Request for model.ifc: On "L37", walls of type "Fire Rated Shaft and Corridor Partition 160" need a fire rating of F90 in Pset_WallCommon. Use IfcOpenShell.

First a look at what the model holds.

```python
import ifcopenshell
import ifcopenshell.util.element

model = ifcopenshell.open("model.ifc")
print(model.schema)
storey = next(s for s in model.by_type("IfcBuildingStorey") if s.Name == "L37")
walls = [e for e in ifcopenshell.util.element.get_decomposition(storey) if e.is_a("IfcWall")]
seen = {}
for e in walls:
    element_type = ifcopenshell.util.element.get_type(e)
    key = (element_type.Name if element_type != e and element_type else None, ifcopenshell.util.element.get_pset(e, "Pset_WallCommon", "FireRating"))
    seen[key] = seen.get(key, 0) + 1
for (name, value), count in sorted(seen.items(), key=str):
    print(count, "x", name, "|", value)
```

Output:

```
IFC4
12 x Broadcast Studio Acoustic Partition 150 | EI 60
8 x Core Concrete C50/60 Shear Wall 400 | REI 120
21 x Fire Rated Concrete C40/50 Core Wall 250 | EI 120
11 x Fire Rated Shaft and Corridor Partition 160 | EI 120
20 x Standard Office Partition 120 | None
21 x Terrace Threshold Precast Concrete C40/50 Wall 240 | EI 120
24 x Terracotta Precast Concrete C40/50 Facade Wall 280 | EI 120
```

```python
import ifcopenshell
import ifcopenshell.api.pset
import ifcopenshell.util.element

model = ifcopenshell.open("model.ifc")

storey = next(s for s in model.by_type("IfcBuildingStorey") if s.Name == "L37")
walls = [e for e in ifcopenshell.util.element.get_decomposition(storey) if e.is_a("IfcWall")]

count = 0
for e in walls:
    element_type = ifcopenshell.util.element.get_type(e)
    if element_type in (None, e) or element_type.Name != "Fire Rated Shaft and Corridor Partition 160":
        continue
    found = ifcopenshell.util.element.get_pset(e, "Pset_WallCommon", should_inherit=False)
    if found:
        pset = model.by_id(found["id"])
        if len(ifcopenshell.util.element.get_elements_by_pset(pset)) > 1:
            pset = ifcopenshell.api.pset.unshare_pset(model, products=[e], pset=pset)[0]
    else:
        pset = ifcopenshell.api.pset.add_pset(model, product=e, name="Pset_WallCommon")
    ifcopenshell.api.pset.edit_pset(model, pset=pset, properties={"FireRating": "F90"})
    count += 1

print(count, "walls updated")

model.write("model_v2.ifc")
```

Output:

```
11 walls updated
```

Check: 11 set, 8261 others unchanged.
